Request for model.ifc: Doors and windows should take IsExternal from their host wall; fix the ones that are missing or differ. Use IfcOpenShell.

First a look at what the model holds.

```python
import ifcopenshell
import ifcopenshell.util.element

model = ifcopenshell.open("model.ifc")
print(model.schema)
seen = {}
for e in model.by_type("IfcDoor") + model.by_type("IfcWindow"):
    if not e.FillsVoids:
        continue
    host = e.FillsVoids[0].RelatingOpeningElement.VoidsElements[0].RelatingBuildingElement
    own = ifcopenshell.util.element.get_pset(e, f"Pset_{e.is_a()[3:].removesuffix('StandardCase')}Common", "IsExternal")
    wall = ifcopenshell.util.element.get_pset(host, "Pset_WallCommon", "IsExternal")
    seen[e.is_a(), own, wall] = seen.get((e.is_a(), own, wall), 0) + 1
for (cls, own, wall), count in sorted(seen.items(), key=str):
    print(count, cls, "IsExternal:", own, "| host wall:", wall)
```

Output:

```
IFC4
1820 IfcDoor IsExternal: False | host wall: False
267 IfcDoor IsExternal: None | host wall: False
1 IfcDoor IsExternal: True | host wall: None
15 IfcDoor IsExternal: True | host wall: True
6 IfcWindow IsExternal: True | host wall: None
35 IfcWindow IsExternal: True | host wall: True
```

```python
import ifcopenshell
import ifcopenshell.api.pset
import ifcopenshell.util.element

model = ifcopenshell.open("model.ifc")

count = 0
for ifc_class, pset_name in (("IfcDoor", "Pset_DoorCommon"), ("IfcWindow", "Pset_WindowCommon")):
    for e in model.by_type(ifc_class):
        if not e.FillsVoids:
            continue
        host = e.FillsVoids[0].RelatingOpeningElement.VoidsElements[0].RelatingBuildingElement
        external = ifcopenshell.util.element.get_pset(host, "Pset_WallCommon", "IsExternal")
        if external is None or ifcopenshell.util.element.get_pset(e, pset_name, "IsExternal") == external:
            continue
        pset = ifcopenshell.api.pset.add_pset(model, product=e, name=pset_name)
        ifcopenshell.api.pset.edit_pset(model, pset=pset, properties={"IsExternal": external})
        count += 1

print(count, "updated")

model.write("model_v2.ifc")
```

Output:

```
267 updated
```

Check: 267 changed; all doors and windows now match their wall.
